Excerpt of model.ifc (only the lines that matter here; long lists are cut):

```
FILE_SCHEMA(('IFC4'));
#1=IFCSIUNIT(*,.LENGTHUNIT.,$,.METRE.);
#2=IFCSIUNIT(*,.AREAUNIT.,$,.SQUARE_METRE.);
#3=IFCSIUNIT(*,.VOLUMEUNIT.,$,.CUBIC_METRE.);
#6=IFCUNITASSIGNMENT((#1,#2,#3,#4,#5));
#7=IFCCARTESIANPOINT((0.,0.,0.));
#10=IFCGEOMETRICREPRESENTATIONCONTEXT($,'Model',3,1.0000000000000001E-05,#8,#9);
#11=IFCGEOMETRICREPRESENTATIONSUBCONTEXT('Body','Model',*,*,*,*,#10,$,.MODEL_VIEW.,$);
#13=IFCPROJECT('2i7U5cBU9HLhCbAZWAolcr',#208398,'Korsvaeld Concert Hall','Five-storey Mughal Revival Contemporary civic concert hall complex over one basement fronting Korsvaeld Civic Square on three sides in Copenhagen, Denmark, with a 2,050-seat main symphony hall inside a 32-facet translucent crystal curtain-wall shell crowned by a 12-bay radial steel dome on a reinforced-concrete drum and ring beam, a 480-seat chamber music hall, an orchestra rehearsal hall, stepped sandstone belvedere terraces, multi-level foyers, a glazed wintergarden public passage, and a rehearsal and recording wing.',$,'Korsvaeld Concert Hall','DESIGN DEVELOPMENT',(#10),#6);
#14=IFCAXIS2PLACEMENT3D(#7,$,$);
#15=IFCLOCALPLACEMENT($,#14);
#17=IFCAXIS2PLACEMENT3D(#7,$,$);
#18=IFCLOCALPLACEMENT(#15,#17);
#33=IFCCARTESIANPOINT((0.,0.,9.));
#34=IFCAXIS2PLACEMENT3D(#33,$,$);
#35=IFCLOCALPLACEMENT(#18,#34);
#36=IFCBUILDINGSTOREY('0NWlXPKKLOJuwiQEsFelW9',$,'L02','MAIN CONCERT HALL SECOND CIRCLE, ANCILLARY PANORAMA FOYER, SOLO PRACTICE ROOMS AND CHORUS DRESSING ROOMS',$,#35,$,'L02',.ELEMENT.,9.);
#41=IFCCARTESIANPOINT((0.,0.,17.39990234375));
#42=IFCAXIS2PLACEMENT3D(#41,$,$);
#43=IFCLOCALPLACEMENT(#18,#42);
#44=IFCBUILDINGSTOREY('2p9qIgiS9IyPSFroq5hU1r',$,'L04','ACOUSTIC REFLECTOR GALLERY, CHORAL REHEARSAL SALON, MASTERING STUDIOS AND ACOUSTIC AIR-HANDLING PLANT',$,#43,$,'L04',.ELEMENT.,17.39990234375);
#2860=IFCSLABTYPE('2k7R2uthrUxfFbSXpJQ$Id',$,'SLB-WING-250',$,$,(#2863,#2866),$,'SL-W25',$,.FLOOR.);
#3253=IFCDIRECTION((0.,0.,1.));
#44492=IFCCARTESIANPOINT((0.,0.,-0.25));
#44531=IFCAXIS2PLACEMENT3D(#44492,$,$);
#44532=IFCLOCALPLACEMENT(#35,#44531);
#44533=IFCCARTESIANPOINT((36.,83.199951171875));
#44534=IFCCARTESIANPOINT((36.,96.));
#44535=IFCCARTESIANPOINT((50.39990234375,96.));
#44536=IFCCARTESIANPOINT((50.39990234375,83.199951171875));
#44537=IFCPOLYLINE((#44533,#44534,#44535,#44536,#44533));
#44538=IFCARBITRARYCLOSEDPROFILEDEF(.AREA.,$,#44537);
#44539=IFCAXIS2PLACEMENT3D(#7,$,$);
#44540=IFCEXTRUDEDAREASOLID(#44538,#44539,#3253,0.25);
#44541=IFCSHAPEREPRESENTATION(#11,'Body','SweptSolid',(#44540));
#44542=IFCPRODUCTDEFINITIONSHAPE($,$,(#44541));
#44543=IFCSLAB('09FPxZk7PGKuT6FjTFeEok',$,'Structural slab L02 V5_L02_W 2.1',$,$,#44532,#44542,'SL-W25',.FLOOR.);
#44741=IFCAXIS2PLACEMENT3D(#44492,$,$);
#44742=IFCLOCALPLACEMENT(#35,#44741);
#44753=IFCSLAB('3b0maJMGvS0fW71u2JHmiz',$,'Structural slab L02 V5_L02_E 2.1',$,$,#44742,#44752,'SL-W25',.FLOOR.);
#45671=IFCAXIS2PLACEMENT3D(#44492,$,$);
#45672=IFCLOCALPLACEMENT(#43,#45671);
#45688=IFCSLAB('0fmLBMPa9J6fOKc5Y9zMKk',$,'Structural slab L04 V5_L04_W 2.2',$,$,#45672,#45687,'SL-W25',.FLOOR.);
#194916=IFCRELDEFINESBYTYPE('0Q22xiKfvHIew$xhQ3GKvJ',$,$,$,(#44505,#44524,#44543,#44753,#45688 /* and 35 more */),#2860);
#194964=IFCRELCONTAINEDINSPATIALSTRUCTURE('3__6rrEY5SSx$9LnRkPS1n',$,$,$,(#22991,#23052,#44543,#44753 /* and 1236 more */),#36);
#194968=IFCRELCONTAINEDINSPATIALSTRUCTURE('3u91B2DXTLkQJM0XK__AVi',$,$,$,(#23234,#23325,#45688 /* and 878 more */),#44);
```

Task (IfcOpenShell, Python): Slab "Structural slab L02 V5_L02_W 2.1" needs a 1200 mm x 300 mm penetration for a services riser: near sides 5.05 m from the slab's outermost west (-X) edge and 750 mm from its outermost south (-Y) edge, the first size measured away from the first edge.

```python
import numpy as np
import ifcopenshell
import ifcopenshell.api.feature
import ifcopenshell.api.geometry
import ifcopenshell.api.root
import ifcopenshell.geom
import ifcopenshell.util.placement
import ifcopenshell.util.representation
import ifcopenshell.util.shape
import ifcopenshell.util.unit

model = ifcopenshell.open("model.ifc")
unit_scale = ifcopenshell.util.unit.calculate_unit_scale(model)
settings = ifcopenshell.geom.settings()


def volume(element):
    """Net volume in cubic metres, openings subtracted."""
    shape = ifcopenshell.geom.create_shape(settings, element)
    return ifcopenshell.util.shape.get_volume(shape.geometry)


slab = model.by_id(44543)
before = volume(slab)

# Extent in the slab's own axes, in metres. The edges named are its -X and -Y sides.
slab_shape = ifcopenshell.geom.create_shape(settings, slab)
vertices = ifcopenshell.util.shape.get_vertices(slab_shape.geometry)
x_min, y_min, bottom = vertices.min(axis=0)
top = vertices[:, 2].max()

opening = ifcopenshell.api.root.create_entity(model, ifc_class="IfcOpeningElement", name="Services riser opening", predefined_type="OPENING")
context = ifcopenshell.util.representation.get_context(model, "Model", "Body", "MODEL_VIEW")
width, depth = 1.2, 0.3
outline = [(0.0, 0.0), (width, 0.0), (width, depth), (0.0, depth), (0.0, 0.0)]
# Overshoot both faces by 50 mm so the cut is clean.
shape = ifcopenshell.api.geometry.add_slab_representation(
    model, context=context, depth=top - bottom + 0.1, polyline=outline
)
ifcopenshell.api.geometry.assign_representation(model, product=opening, representation=shape)

matrix = ifcopenshell.util.placement.get_local_placement(slab.ObjectPlacement)
matrix[:, 3] = matrix @ np.append(np.array([x_min + 5.05, y_min + 0.75, bottom - 0.05]) / unit_scale, 1.0)
ifcopenshell.api.geometry.edit_object_placement(model, product=opening, matrix=matrix, is_si=False)
ifcopenshell.api.feature.add_feature(model, feature=opening, element=slab)

after = volume(slab)

print(f"slab volume {before:.3f} -> {after:.3f} m3")

model.write("model_updated.ifc")
```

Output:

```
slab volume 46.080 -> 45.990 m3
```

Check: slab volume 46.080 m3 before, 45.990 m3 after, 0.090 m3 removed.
